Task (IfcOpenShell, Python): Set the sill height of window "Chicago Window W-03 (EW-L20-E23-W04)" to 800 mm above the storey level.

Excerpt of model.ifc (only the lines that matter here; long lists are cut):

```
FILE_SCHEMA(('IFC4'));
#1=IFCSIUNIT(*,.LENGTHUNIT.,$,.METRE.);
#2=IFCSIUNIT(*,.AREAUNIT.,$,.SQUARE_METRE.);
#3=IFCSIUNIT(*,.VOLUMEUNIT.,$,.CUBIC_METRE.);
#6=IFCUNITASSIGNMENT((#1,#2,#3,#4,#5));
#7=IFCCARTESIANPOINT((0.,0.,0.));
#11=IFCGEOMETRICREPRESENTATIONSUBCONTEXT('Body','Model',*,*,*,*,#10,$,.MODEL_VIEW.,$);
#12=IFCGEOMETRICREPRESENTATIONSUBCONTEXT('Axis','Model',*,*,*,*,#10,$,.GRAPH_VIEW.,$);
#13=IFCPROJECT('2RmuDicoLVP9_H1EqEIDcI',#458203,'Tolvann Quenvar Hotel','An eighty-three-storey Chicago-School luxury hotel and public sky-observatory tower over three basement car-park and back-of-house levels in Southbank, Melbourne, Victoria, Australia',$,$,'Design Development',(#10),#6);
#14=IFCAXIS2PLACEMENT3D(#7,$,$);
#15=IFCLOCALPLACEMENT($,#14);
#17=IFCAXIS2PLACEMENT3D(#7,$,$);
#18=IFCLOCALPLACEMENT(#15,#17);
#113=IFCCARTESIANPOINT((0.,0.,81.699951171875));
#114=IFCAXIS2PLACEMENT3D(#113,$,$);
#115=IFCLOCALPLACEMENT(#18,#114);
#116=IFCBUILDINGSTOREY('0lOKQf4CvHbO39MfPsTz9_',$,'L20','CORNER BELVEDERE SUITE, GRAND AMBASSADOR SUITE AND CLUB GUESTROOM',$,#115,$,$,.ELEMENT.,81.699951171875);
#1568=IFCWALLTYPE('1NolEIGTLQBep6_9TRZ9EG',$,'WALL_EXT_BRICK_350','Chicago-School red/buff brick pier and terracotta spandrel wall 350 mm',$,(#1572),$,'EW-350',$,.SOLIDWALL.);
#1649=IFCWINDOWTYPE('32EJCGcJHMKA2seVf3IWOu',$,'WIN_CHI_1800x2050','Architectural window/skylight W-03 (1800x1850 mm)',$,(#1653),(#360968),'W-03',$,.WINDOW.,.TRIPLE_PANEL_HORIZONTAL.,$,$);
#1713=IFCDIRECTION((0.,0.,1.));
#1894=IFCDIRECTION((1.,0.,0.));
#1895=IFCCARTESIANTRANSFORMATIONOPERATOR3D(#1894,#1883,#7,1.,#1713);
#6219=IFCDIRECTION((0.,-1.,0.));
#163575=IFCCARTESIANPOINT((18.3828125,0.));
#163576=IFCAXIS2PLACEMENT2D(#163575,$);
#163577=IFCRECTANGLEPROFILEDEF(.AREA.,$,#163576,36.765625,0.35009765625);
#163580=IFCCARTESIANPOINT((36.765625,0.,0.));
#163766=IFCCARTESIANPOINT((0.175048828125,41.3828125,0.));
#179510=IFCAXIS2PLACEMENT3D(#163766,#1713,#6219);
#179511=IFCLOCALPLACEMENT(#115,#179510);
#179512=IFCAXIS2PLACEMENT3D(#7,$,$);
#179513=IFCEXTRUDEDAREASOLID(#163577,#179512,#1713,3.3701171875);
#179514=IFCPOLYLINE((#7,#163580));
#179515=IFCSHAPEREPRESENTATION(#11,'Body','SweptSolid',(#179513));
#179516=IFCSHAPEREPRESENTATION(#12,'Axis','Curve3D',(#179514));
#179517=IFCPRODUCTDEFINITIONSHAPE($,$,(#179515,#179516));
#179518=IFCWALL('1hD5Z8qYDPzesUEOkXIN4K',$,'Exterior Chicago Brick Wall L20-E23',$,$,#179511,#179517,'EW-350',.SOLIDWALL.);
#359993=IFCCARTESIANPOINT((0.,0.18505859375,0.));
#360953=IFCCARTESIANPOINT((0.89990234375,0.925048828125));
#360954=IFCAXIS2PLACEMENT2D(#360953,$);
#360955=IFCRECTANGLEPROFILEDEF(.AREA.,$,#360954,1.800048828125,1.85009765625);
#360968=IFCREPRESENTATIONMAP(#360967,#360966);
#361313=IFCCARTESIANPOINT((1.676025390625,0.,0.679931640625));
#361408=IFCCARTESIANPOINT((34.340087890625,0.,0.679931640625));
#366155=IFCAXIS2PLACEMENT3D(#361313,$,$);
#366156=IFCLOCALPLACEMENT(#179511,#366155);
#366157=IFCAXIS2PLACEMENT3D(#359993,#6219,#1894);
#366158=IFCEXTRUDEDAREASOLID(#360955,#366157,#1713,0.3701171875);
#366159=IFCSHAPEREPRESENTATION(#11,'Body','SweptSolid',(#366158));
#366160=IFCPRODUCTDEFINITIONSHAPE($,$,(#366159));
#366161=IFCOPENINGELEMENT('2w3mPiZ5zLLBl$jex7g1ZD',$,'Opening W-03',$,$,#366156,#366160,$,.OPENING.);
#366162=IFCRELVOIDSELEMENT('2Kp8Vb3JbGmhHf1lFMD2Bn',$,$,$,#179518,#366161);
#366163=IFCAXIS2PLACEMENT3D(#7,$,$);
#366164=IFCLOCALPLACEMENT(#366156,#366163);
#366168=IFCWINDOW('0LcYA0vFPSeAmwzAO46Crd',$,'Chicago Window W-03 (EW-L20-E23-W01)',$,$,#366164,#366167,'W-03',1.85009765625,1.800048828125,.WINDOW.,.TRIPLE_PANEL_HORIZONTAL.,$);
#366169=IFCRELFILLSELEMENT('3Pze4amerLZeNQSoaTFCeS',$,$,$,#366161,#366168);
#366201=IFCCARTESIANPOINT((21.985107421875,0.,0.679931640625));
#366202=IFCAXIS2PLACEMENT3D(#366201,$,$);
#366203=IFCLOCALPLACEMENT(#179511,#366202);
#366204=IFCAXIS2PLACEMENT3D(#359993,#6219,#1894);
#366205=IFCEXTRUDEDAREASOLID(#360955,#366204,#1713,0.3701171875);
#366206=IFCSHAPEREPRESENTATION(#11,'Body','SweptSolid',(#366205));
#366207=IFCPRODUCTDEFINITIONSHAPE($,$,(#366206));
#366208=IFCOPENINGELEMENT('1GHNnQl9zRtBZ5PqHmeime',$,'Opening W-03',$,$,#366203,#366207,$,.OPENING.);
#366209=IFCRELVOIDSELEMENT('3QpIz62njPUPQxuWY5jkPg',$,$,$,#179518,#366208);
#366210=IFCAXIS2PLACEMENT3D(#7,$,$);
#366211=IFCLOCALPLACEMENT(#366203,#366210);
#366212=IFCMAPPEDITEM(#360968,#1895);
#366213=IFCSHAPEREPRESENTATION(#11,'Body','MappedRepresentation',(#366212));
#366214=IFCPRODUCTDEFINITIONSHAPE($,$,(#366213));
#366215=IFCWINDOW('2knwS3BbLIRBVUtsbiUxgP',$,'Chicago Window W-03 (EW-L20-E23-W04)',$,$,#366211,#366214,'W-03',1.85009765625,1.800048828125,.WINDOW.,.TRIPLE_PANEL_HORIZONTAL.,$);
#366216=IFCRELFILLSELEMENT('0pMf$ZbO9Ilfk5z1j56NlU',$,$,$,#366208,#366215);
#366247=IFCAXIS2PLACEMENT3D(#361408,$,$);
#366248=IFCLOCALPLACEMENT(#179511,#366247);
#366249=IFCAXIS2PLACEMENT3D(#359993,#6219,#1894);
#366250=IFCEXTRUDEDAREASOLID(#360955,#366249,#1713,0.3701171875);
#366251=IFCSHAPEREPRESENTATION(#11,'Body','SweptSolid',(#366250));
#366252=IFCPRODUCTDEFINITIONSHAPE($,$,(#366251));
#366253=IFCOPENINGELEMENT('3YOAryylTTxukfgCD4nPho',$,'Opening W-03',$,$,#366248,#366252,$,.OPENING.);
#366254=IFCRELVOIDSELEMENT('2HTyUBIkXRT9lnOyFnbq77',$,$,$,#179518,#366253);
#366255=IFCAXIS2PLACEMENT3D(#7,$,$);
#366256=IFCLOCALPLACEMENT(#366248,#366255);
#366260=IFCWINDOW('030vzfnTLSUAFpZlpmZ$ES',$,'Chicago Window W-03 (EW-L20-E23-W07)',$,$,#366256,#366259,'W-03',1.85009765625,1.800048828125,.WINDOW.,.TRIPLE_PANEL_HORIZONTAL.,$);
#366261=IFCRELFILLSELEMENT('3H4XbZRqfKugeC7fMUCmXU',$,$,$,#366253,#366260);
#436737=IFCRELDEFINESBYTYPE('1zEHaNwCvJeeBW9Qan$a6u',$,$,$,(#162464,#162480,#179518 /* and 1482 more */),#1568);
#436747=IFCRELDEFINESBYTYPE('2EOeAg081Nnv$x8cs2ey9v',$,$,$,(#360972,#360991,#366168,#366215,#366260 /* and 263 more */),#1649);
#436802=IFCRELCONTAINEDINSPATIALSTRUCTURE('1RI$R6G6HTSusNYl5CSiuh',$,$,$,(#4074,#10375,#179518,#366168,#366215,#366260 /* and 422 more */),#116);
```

```python
import numpy as np
import ifcopenshell
import ifcopenshell.api.geometry
import ifcopenshell.geom
import ifcopenshell.util.element
import ifcopenshell.util.placement
import ifcopenshell.util.shape
import ifcopenshell.util.unit

model = ifcopenshell.open("model.ifc")
unit_scale = ifcopenshell.util.unit.calculate_unit_scale(model)

window = model.by_guid("2knwS3BbLIRBVUtsbiUxgP")
opening = window.FillsVoids[0].RelatingOpeningElement
storey = ifcopenshell.util.element.get_container(window, ifc_class="IfcBuildingStorey")
level = ifcopenshell.util.placement.get_local_placement(storey.ObjectPlacement)[2, 3]

# The opening's origin need not be at the sill, so measure its lowest point.
shape = ifcopenshell.geom.create_shape(ifcopenshell.geom.settings(), opening)
bottom = ifcopenshell.util.shape.get_shape_bottom_elevation(shape, shape.geometry) / unit_scale
dz = level + 0.8 - bottom

shift = np.array([0.0, 0.0, dz])
# The window is placed relative to its opening, so it follows when the opening moves.
matrix = ifcopenshell.util.placement.get_local_placement(opening.ObjectPlacement)
matrix[:3, 3] += shift
ifcopenshell.api.geometry.edit_object_placement(
    model, product=opening, matrix=matrix, is_si=False, should_transform_children=True
)

print(f"moved by {dz * unit_scale:+.3f} m")

model.write("model_updated.ifc")
```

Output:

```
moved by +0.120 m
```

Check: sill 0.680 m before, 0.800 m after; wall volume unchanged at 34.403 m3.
